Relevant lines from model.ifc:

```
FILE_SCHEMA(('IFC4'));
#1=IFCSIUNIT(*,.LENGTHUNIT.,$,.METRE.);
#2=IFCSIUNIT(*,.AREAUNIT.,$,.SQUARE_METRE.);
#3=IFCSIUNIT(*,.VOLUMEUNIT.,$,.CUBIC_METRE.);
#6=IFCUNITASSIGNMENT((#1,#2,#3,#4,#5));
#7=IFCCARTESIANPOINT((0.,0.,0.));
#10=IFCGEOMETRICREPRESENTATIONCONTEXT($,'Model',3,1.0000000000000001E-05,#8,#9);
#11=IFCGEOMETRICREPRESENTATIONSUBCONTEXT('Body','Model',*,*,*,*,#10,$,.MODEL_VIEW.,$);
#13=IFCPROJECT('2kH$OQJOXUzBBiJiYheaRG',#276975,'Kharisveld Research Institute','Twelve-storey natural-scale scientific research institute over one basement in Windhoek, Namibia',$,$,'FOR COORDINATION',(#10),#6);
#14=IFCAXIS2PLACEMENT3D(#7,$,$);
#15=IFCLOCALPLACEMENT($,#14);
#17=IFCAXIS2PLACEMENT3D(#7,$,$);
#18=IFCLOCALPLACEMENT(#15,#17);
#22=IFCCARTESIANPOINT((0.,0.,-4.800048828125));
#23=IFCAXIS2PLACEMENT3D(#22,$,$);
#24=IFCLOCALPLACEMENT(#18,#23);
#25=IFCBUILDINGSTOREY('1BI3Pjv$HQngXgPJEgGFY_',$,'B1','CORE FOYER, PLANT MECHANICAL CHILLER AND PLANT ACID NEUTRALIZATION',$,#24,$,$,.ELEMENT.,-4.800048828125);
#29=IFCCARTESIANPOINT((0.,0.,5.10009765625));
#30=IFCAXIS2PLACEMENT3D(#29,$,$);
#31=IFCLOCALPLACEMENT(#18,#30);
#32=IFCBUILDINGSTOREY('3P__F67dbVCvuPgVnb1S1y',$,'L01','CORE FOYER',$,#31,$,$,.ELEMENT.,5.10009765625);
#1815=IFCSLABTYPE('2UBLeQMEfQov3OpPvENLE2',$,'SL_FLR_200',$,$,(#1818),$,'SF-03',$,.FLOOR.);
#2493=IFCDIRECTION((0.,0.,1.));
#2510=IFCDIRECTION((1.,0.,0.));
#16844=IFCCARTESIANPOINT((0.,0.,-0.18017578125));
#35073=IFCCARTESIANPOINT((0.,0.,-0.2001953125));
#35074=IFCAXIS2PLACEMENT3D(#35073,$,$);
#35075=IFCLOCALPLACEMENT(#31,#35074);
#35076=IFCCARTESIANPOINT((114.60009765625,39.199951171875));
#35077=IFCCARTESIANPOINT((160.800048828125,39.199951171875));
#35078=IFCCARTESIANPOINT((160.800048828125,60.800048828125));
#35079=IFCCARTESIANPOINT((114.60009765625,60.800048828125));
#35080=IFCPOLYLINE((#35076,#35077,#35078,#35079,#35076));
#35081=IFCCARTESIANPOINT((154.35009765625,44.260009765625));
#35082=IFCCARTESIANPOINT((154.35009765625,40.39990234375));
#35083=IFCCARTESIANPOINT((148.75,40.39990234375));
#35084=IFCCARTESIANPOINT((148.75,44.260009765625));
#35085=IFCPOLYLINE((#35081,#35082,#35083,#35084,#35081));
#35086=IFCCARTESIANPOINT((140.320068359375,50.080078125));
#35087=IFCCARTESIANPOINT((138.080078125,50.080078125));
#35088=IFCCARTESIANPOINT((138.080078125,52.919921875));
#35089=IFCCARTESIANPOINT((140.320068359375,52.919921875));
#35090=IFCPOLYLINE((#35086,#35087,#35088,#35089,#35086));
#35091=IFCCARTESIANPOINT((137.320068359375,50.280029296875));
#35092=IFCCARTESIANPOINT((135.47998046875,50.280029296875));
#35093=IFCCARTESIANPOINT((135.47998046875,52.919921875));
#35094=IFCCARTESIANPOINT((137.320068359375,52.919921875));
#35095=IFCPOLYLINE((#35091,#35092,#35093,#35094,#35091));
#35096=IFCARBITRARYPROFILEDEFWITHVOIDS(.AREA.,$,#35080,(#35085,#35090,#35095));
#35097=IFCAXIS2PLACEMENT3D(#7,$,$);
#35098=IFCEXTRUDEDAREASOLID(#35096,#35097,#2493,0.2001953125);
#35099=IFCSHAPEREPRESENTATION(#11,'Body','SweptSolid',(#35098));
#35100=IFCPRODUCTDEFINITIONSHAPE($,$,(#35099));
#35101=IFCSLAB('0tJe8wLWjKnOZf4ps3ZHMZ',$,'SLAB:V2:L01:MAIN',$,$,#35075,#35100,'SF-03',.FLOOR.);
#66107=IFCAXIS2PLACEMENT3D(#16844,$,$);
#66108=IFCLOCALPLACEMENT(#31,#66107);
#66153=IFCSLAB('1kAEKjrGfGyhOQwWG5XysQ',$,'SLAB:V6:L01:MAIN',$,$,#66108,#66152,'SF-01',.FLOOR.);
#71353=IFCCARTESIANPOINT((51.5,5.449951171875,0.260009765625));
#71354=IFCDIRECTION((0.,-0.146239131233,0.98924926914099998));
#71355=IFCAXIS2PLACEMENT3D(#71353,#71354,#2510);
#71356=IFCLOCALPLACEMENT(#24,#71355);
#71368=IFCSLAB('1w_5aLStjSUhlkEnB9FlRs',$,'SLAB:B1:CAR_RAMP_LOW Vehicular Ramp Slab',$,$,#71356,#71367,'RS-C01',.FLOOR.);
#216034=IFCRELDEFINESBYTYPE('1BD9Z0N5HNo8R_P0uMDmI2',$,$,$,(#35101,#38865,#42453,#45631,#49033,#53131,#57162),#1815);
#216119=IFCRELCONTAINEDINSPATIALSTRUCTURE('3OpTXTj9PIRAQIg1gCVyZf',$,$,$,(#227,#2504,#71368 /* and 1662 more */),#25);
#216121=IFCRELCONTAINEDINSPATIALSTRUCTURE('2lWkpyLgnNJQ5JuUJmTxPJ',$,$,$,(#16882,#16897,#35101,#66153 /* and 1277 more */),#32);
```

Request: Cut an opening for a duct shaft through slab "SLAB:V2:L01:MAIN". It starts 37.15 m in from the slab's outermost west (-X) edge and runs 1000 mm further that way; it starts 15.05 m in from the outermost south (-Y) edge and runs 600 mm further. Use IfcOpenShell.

```python
import numpy as np
import ifcopenshell
import ifcopenshell.api.feature
import ifcopenshell.api.geometry
import ifcopenshell.api.root
import ifcopenshell.geom
import ifcopenshell.util.placement
import ifcopenshell.util.representation
import ifcopenshell.util.shape
import ifcopenshell.util.unit

model = ifcopenshell.open("model.ifc")
unit_scale = ifcopenshell.util.unit.calculate_unit_scale(model)
settings = ifcopenshell.geom.settings()


def volume(element):
    """Net volume in cubic metres, openings subtracted."""
    shape = ifcopenshell.geom.create_shape(settings, element)
    return ifcopenshell.util.shape.get_volume(shape.geometry)


slab = model.by_guid("0tJe8wLWjKnOZf4ps3ZHMZ")
before = volume(slab)

# Extent in the slab's own axes, in metres. The edges named are its -X and -Y sides.
slab_shape = ifcopenshell.geom.create_shape(settings, slab)
vertices = ifcopenshell.util.shape.get_vertices(slab_shape.geometry)
x_min, y_min, bottom = vertices.min(axis=0)
top = vertices[:, 2].max()

opening = ifcopenshell.api.root.create_entity(model, ifc_class="IfcOpeningElement", name="Duct shaft opening", predefined_type="OPENING")
context = ifcopenshell.util.representation.get_context(model, "Model", "Body", "MODEL_VIEW")
width, depth = 1, 0.6
outline = [(0.0, 0.0), (width, 0.0), (width, depth), (0.0, depth), (0.0, 0.0)]
# Overshoot both faces by 50 mm so the cut is clean.
shape = ifcopenshell.api.geometry.add_slab_representation(
    model, context=context, depth=top - bottom + 0.1, polyline=outline
)
ifcopenshell.api.geometry.assign_representation(model, product=opening, representation=shape)

matrix = ifcopenshell.util.placement.get_local_placement(slab.ObjectPlacement)
matrix[:, 3] = matrix @ np.append(np.array([x_min + 37.15, y_min + 15.05, bottom - 0.05]) / unit_scale, 1.0)
ifcopenshell.api.geometry.edit_object_placement(model, product=opening, matrix=matrix, is_si=False)
ifcopenshell.api.feature.add_feature(model, feature=opening, element=slab)

after = volume(slab)

print(f"slab volume {before:.3f} -> {after:.3f} m3")

model.write("model_v2.ifc")
```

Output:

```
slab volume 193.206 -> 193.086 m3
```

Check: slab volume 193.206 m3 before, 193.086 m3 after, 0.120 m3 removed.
